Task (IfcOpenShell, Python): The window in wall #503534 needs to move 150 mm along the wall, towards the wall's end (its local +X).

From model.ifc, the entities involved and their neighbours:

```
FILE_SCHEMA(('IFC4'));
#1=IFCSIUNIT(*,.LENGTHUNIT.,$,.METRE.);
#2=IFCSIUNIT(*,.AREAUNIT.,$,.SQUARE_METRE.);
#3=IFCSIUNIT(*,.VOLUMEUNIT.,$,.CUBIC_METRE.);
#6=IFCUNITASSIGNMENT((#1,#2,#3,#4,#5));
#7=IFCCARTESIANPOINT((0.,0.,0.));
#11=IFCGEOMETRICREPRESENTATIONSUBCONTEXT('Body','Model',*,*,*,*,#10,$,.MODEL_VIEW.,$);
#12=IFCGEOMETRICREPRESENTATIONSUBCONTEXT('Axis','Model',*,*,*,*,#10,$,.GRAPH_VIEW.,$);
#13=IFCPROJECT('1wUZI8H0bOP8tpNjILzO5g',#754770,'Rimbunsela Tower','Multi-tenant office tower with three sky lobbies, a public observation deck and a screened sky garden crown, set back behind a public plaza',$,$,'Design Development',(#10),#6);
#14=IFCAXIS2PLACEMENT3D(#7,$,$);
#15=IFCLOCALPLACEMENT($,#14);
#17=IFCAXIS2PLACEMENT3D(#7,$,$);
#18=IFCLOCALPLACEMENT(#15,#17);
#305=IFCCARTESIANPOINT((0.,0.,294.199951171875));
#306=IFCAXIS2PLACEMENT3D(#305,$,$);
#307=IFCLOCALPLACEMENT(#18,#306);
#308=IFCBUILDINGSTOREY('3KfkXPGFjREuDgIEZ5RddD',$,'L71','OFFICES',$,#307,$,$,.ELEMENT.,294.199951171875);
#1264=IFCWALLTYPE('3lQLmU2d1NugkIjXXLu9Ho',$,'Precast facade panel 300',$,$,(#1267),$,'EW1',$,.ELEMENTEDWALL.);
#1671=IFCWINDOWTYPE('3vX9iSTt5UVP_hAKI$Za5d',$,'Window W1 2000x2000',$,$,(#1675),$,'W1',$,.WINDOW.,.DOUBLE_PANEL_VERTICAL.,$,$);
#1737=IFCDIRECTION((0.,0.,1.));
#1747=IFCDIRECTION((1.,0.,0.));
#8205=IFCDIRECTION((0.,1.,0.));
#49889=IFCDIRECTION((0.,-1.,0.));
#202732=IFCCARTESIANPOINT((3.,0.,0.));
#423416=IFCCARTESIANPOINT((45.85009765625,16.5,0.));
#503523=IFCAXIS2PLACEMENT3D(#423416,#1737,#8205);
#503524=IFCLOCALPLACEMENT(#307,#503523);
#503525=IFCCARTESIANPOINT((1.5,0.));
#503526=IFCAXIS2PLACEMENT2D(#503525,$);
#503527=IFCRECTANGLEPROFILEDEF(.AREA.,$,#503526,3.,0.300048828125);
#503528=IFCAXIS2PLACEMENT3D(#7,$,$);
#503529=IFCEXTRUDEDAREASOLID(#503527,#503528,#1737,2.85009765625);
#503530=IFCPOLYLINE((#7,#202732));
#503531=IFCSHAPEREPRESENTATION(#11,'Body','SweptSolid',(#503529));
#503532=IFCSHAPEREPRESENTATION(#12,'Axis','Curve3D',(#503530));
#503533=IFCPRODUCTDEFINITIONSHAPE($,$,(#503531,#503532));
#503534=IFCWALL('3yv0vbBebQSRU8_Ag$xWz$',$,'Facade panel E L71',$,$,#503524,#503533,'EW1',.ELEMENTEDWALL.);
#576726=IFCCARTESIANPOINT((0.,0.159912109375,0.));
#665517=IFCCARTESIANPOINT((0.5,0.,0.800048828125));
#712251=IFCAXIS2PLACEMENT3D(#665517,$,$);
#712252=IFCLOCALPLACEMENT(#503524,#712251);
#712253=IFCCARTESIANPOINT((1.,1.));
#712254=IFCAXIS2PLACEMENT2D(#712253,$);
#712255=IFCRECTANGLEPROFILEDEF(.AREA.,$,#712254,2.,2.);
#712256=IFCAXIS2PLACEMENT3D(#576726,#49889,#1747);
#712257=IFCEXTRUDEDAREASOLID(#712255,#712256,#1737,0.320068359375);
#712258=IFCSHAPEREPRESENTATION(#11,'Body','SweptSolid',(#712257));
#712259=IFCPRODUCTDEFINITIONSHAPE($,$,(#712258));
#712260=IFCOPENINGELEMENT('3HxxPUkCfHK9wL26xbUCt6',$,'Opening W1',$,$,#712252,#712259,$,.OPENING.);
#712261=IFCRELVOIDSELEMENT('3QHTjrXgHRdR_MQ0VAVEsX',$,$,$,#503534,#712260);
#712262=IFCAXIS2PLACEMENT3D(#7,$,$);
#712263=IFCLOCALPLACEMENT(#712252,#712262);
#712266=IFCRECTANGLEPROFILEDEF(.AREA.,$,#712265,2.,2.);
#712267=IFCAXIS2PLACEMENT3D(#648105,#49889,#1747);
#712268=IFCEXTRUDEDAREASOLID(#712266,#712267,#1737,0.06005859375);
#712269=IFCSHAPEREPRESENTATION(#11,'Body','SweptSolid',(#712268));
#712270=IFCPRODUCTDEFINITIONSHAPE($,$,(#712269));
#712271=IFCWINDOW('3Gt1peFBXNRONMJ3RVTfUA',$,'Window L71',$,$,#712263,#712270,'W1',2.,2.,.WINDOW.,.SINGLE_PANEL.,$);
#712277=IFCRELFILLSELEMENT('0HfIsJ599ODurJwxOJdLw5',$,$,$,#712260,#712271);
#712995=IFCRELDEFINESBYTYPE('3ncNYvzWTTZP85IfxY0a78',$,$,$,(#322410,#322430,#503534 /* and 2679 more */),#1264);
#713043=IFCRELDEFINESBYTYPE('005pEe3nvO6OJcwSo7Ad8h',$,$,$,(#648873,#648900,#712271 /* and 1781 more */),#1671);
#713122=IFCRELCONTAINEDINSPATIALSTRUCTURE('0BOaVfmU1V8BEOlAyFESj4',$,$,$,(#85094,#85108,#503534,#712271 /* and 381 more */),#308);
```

```python
import ifcopenshell
import ifcopenshell.api.geometry
import ifcopenshell.util.placement

model = ifcopenshell.open("model.ifc")

window = model.by_id(712271)
opening = window.FillsVoids[0].RelatingOpeningElement
wall = opening.VoidsElements[0].RelatingBuildingElement

wall_matrix = ifcopenshell.util.placement.get_local_placement(wall.ObjectPlacement)
shift = wall_matrix[:3, 0] * 0.15
before = ifcopenshell.util.placement.get_local_placement(window.ObjectPlacement)[:3, 3].copy()

# The window is placed relative to its opening, so it follows when the opening moves.
matrix = ifcopenshell.util.placement.get_local_placement(opening.ObjectPlacement)
matrix[:3, 3] += shift
ifcopenshell.api.geometry.edit_object_placement(
    model, product=opening, matrix=matrix, is_si=False, should_transform_children=True
)

after = ifcopenshell.util.placement.get_local_placement(window.ObjectPlacement)[:3, 3]
print("window moved by", (after - before).round(3) + 0.0)

model.write("model_rev.ifc")
```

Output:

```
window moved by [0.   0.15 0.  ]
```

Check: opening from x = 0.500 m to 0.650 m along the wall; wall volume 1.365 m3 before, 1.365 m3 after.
